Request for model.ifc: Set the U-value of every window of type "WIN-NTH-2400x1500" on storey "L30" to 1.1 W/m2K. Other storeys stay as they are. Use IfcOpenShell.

First a look at what the model holds.

```python
import ifcopenshell
import ifcopenshell.util.element

model = ifcopenshell.open("model.ifc")
print(model.schema)
storey = next(s for s in model.by_type("IfcBuildingStorey") if s.Name == "L30")
windows = [e for e in ifcopenshell.util.element.get_decomposition(storey) if e.is_a("IfcWindow")]
seen = {}
for e in windows:
    element_type = ifcopenshell.util.element.get_type(e)
    key = (element_type.Name if element_type != e and element_type else None, ifcopenshell.util.element.get_pset(e, "Pset_WindowCommon", "ThermalTransmittance"))
    seen[key] = seen.get(key, 0) + 1
for (name, value), count in sorted(seen.items(), key=str):
    print(count, "x", name, "|", value)
```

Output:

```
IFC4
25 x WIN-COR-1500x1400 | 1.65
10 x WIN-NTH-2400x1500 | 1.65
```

```python
import ifcopenshell
import ifcopenshell.api.pset
import ifcopenshell.util.element

model = ifcopenshell.open("model.ifc")

storey = next(s for s in model.by_type("IfcBuildingStorey") if s.Name == "L30")
windows = [e for e in ifcopenshell.util.element.get_decomposition(storey) if e.is_a("IfcWindow")]

count = 0
for e in windows:
    element_type = ifcopenshell.util.element.get_type(e)
    if element_type in (None, e) or element_type.Name != "WIN-NTH-2400x1500":
        continue
    # add_pset returns the element's existing set when there is one.
    pset = ifcopenshell.api.pset.add_pset(model, product=e, name="Pset_WindowCommon")
    ifcopenshell.api.pset.edit_pset(model, pset=pset, properties={"ThermalTransmittance": 1.1})
    count += 1

print(count, "windows updated")

model.write("model_edited.ifc")
```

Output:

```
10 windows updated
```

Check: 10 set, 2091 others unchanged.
